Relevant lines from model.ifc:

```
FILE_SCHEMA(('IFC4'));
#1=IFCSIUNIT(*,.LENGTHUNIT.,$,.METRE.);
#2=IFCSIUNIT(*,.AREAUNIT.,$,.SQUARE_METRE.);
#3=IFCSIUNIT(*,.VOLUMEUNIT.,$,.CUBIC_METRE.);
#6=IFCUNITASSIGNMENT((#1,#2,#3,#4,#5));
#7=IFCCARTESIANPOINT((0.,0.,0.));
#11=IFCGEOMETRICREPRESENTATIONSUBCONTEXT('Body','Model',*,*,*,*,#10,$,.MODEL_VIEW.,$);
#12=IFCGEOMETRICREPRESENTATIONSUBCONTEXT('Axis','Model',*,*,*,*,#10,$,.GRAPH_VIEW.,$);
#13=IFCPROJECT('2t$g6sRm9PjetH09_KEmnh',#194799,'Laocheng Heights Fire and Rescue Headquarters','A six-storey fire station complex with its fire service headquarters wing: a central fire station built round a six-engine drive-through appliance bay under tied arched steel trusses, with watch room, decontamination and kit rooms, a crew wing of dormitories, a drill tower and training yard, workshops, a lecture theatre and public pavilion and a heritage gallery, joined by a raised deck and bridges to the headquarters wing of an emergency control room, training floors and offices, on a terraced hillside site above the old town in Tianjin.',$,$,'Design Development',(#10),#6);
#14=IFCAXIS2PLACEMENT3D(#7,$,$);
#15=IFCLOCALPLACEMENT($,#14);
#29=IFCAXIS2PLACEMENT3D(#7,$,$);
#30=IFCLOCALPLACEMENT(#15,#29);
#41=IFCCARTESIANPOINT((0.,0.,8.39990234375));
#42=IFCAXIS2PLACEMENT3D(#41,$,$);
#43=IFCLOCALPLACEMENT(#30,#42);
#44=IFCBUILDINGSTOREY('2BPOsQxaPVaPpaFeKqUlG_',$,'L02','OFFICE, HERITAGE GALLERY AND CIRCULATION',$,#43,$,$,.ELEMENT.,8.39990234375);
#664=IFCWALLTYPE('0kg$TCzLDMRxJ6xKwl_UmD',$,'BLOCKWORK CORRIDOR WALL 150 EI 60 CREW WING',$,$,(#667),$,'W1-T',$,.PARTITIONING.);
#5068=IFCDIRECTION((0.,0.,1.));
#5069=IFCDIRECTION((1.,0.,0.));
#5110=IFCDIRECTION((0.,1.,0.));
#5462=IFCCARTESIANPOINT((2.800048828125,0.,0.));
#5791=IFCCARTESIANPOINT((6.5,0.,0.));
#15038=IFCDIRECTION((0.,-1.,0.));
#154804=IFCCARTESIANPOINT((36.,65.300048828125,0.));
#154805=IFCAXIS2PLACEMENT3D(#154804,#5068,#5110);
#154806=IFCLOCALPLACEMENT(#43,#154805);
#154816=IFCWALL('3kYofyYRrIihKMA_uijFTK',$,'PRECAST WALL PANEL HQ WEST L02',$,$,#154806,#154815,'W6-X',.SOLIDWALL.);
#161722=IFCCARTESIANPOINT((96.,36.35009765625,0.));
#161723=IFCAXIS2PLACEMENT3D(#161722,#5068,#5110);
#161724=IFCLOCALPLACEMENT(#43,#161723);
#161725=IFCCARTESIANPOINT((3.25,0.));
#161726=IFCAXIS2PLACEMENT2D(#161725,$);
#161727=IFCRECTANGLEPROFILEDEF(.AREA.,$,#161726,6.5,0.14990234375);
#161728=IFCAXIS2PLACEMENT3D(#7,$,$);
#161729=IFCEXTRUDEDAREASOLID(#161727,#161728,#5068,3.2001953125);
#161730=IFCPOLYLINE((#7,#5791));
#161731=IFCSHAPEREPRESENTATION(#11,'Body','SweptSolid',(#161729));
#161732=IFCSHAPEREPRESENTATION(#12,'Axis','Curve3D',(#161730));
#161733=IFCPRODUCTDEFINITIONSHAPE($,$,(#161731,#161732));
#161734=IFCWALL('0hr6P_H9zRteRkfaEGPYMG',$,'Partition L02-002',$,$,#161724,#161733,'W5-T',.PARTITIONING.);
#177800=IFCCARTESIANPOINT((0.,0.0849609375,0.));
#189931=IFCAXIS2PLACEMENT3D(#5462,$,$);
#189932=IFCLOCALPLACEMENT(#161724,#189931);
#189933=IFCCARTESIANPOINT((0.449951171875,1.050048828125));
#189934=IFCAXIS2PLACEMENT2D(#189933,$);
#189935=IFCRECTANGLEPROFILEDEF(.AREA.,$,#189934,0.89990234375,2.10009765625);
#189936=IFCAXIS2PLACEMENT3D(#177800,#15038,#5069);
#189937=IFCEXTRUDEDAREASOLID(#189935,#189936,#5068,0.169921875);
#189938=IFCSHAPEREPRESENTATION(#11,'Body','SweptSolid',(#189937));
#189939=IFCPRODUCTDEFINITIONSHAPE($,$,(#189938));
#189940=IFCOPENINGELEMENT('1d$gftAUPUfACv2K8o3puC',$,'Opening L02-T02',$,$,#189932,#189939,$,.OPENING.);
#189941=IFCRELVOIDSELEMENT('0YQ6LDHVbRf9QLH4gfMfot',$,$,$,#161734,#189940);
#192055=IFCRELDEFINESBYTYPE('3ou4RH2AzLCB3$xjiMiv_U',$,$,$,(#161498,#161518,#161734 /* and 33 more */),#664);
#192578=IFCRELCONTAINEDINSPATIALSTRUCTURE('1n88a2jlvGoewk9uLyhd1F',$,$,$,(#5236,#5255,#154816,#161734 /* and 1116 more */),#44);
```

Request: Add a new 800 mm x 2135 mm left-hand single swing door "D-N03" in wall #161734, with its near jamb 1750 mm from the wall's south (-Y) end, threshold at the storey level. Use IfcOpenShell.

```python
import numpy as np
import ifcopenshell
import ifcopenshell.api.feature
import ifcopenshell.api.geometry
import ifcopenshell.api.root
import ifcopenshell.api.spatial
import ifcopenshell.geom
import ifcopenshell.util.element
import ifcopenshell.util.placement
import ifcopenshell.util.representation
import ifcopenshell.util.shape
import ifcopenshell.util.unit

model = ifcopenshell.open("model.ifc")
unit_scale = ifcopenshell.util.unit.calculate_unit_scale(model)
settings = ifcopenshell.geom.settings()


def volume(element):
    """Net volume in cubic metres, openings subtracted."""
    shape = ifcopenshell.geom.create_shape(settings, element)
    return ifcopenshell.util.shape.get_volume(shape.geometry)


wall = model.by_guid("0hr6P_H9zRteRkfaEGPYMG")
storey = ifcopenshell.util.element.get_container(wall, ifc_class="IfcBuildingStorey")
context = ifcopenshell.util.representation.get_context(model, "Model", "Body", "MODEL_VIEW")
before = volume(wall)

width, height, from_end, sill = 0.8, 2.135, 1.75, 0.0  # metres

# The wall runs along its own X axis, and the end named is its -X end.
wall_shape = ifcopenshell.geom.create_shape(settings, wall)
x, y, z = ifcopenshell.util.shape.get_vertices(wall_shape.geometry).T
start = x.min() + from_end
face, thickness = float(y.min()), float(y.max() - y.min())
wall_matrix = ifcopenshell.util.placement.get_local_placement(wall.ObjectPlacement)
level = ifcopenshell.util.placement.get_local_placement(storey.ObjectPlacement)[2, 3]


def in_wall(x, y):
    """Placement at x, y metres in the wall's axes, at sill height."""
    matrix = wall_matrix.copy()
    matrix[:, 3] = wall_matrix @ np.array([x / unit_scale, y / unit_scale, 0.0, 1.0])
    matrix[2, 3] = level + sill / unit_scale
    return matrix


# Opening: a box that overshoots both wall faces by 50 mm.
opening = ifcopenshell.api.root.create_entity(model, ifc_class="IfcOpeningElement", predefined_type="OPENING")
box = ifcopenshell.api.geometry.add_wall_representation(
    model, context=context, length=width, height=height, thickness=thickness + 0.1
)
ifcopenshell.api.geometry.assign_representation(model, product=opening, representation=box)
ifcopenshell.api.geometry.edit_object_placement(model, product=opening, matrix=in_wall(start, face - 0.05), is_si=False)
ifcopenshell.api.feature.add_feature(model, feature=opening, element=wall)

door = ifcopenshell.api.root.create_entity(model, ifc_class="IfcDoor", name="D-N03", predefined_type="DOOR")
door.OverallWidth, door.OverallHeight = width / unit_scale, height / unit_scale
door.OperationType = "SINGLE_SWING_LEFT"
body = ifcopenshell.api.geometry.add_door_representation(
    model,
    context=context,
    overall_width=door.OverallWidth,
    overall_height=door.OverallHeight,
    operation_type="SINGLE_SWING_LEFT",
    lining_properties={"LiningDepth": thickness / unit_scale, "ThresholdDepth": thickness / unit_scale},
)
ifcopenshell.api.geometry.assign_representation(model, product=door, representation=body)
ifcopenshell.api.spatial.assign_container(model, products=[door], relating_structure=storey)
ifcopenshell.api.feature.add_filling(model, opening=opening, element=door)

# The lining spans the wall, so the door starts at the wall face.
ifcopenshell.api.geometry.edit_object_placement(model, product=door, matrix=in_wall(start, face), is_si=False)

after = volume(wall)

print(f"wall volume {before:.3f} -> {after:.3f} m3")

model.write("model_rev.ifc")
```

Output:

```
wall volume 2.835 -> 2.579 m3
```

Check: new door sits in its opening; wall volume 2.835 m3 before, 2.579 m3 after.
